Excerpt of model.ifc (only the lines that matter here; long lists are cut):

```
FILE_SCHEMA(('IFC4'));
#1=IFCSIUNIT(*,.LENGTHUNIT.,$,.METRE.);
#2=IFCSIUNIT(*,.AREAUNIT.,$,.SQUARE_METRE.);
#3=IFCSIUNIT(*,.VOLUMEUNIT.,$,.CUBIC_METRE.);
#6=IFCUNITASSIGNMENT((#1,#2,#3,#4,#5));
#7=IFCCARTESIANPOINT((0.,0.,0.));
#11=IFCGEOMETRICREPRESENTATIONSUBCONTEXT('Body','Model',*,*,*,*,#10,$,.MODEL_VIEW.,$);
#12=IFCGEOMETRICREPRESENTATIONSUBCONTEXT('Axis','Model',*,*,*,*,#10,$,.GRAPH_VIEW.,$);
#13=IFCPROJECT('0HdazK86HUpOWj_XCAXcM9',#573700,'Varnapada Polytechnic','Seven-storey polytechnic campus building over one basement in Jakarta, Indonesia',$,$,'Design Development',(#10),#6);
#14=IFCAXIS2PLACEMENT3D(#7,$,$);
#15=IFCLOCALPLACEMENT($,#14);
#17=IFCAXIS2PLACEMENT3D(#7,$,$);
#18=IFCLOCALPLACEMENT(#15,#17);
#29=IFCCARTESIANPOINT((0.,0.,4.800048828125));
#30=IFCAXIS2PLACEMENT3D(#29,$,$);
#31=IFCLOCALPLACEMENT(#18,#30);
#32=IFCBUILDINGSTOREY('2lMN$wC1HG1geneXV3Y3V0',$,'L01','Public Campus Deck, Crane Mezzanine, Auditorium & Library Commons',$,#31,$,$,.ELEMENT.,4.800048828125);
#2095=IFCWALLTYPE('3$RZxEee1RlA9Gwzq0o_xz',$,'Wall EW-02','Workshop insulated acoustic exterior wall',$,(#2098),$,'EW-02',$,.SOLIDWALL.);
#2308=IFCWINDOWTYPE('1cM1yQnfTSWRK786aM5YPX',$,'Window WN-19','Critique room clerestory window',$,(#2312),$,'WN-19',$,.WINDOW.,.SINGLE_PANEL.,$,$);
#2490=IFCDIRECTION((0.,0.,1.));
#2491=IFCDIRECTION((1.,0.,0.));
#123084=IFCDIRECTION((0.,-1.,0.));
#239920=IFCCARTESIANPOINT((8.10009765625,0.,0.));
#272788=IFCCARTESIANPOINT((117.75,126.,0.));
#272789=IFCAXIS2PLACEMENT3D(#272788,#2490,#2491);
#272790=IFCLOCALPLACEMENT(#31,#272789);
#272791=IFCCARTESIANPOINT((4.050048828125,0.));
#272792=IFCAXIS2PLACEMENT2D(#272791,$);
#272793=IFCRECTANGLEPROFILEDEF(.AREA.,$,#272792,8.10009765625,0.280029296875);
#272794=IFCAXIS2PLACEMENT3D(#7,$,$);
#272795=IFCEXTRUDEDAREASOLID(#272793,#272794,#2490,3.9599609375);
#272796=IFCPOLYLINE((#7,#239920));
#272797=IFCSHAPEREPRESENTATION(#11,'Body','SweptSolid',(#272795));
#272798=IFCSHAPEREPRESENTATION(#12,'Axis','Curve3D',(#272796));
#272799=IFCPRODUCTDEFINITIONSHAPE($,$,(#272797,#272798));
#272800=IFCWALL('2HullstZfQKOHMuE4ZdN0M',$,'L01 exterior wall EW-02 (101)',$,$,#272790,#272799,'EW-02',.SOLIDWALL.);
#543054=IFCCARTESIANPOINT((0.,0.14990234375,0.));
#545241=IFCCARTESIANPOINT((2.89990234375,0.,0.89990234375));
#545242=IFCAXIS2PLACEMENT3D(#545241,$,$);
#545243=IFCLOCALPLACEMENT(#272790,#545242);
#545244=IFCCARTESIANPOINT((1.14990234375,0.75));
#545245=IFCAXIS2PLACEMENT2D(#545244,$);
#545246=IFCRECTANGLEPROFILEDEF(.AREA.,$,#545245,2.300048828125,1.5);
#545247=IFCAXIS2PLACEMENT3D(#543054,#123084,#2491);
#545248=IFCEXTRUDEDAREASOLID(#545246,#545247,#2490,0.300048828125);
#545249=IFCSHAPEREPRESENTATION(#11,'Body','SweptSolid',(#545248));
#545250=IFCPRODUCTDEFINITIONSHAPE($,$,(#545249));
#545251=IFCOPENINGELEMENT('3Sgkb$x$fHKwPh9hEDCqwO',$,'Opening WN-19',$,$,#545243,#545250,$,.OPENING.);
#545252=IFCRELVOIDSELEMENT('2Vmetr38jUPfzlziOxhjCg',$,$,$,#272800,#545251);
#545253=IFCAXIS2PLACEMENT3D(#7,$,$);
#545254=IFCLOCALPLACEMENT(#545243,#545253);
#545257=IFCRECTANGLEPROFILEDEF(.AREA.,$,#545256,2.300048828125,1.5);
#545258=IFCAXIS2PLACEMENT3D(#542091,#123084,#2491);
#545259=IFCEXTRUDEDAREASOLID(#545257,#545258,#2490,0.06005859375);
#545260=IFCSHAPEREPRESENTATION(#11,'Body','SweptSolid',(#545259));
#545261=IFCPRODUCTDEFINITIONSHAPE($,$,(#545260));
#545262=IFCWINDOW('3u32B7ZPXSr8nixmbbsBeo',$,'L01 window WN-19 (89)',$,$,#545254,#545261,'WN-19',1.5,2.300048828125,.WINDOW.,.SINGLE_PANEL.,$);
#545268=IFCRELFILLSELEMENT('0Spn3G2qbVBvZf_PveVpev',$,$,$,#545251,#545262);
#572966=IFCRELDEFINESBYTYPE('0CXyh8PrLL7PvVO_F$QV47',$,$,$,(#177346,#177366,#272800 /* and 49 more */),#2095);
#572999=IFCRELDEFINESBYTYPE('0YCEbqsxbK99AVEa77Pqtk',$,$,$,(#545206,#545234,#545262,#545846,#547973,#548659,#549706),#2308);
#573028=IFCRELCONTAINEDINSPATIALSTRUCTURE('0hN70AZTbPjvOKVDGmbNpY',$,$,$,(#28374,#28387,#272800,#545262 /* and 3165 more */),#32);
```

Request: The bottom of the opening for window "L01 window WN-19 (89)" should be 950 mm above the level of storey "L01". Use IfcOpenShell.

```python
import numpy as np
import ifcopenshell
import ifcopenshell.api.geometry
import ifcopenshell.geom
import ifcopenshell.util.element
import ifcopenshell.util.placement
import ifcopenshell.util.shape
import ifcopenshell.util.unit

model = ifcopenshell.open("model.ifc")
unit_scale = ifcopenshell.util.unit.calculate_unit_scale(model)

window = model.by_guid("3u32B7ZPXSr8nixmbbsBeo")
opening = window.FillsVoids[0].RelatingOpeningElement
storey = ifcopenshell.util.element.get_container(window, ifc_class="IfcBuildingStorey")
level = ifcopenshell.util.placement.get_local_placement(storey.ObjectPlacement)[2, 3]

# The opening's origin need not be at the sill, so measure its lowest point.
shape = ifcopenshell.geom.create_shape(ifcopenshell.geom.settings(), opening)
bottom = ifcopenshell.util.shape.get_shape_bottom_elevation(shape, shape.geometry) / unit_scale
dz = level + 0.95 / unit_scale - bottom

shift = np.array([0.0, 0.0, dz])
# The window is placed relative to its opening, so it follows when the opening moves.
matrix = ifcopenshell.util.placement.get_local_placement(opening.ObjectPlacement)
matrix[:3, 3] += shift
ifcopenshell.api.geometry.edit_object_placement(
    model, product=opening, matrix=matrix, is_si=False, should_transform_children=True
)

print(f"moved by {dz * unit_scale:+.3f} m")

model.write("model_rev.ifc")
```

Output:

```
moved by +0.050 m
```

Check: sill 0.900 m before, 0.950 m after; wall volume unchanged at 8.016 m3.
